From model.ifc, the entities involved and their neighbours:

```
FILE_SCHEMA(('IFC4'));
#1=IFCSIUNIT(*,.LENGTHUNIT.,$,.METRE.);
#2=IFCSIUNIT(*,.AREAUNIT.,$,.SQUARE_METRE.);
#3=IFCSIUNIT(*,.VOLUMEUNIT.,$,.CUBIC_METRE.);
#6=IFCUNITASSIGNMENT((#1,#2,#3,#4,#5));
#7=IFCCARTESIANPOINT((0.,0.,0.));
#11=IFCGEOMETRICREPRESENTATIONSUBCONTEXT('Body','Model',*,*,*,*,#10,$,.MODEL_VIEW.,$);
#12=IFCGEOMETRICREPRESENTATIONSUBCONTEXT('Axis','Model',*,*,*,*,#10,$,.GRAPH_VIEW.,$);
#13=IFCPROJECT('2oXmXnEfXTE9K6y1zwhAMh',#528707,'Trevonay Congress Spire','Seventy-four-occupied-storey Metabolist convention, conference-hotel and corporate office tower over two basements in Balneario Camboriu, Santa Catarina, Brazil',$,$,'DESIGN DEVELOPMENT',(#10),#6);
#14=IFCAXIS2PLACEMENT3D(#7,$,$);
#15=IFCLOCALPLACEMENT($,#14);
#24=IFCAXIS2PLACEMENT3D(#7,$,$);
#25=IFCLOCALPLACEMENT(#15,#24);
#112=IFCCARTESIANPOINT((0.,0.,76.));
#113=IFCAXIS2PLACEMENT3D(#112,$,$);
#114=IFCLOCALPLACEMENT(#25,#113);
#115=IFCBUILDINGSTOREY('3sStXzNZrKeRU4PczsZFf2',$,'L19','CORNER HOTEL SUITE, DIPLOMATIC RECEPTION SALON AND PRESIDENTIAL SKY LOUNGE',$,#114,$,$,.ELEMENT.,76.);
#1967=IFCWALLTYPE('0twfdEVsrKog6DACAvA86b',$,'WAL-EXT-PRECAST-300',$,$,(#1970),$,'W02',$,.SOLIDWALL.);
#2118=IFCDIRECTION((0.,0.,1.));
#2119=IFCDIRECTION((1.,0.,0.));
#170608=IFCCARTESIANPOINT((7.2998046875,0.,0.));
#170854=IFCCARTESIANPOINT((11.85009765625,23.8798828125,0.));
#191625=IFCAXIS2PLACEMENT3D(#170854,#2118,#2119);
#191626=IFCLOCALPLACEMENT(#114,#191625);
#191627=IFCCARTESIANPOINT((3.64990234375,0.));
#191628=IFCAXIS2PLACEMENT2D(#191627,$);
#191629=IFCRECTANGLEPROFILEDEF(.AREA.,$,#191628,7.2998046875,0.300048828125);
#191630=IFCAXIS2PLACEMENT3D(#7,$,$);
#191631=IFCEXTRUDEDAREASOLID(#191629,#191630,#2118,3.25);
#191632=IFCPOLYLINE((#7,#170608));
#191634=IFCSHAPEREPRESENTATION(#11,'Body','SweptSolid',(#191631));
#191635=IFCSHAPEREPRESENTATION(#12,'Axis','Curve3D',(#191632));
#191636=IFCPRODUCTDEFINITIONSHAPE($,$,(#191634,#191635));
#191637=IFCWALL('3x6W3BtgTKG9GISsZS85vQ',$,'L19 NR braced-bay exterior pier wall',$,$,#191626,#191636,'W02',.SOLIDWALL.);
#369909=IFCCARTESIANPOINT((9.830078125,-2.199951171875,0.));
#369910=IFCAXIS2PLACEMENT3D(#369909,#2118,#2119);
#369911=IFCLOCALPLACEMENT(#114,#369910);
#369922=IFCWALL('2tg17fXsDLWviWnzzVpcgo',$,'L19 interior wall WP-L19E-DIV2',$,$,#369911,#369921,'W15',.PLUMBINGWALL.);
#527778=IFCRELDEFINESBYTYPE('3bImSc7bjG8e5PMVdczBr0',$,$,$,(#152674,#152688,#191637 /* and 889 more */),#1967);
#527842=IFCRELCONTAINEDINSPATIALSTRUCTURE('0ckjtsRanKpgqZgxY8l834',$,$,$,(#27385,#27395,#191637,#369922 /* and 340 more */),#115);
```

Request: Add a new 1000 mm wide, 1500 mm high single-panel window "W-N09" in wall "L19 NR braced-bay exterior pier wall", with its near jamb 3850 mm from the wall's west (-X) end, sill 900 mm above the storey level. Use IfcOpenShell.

```python
import numpy as np
import ifcopenshell
import ifcopenshell.api.feature
import ifcopenshell.api.geometry
import ifcopenshell.api.root
import ifcopenshell.api.spatial
import ifcopenshell.geom
import ifcopenshell.util.element
import ifcopenshell.util.placement
import ifcopenshell.util.representation
import ifcopenshell.util.shape
import ifcopenshell.util.unit

model = ifcopenshell.open("model.ifc")
unit_scale = ifcopenshell.util.unit.calculate_unit_scale(model)
settings = ifcopenshell.geom.settings()


def volume(element):
    """Net volume in cubic metres, openings subtracted."""
    shape = ifcopenshell.geom.create_shape(settings, element)
    return ifcopenshell.util.shape.get_volume(shape.geometry)


wall = model.by_guid("3x6W3BtgTKG9GISsZS85vQ")
storey = ifcopenshell.util.element.get_container(wall, ifc_class="IfcBuildingStorey")
context = ifcopenshell.util.representation.get_context(model, "Model", "Body", "MODEL_VIEW")
before = volume(wall)

width, height, from_end, sill = 1, 1.5, 3.85, 0.9  # metres

# The wall runs along its own X axis, and the end named is its -X end.
wall_shape = ifcopenshell.geom.create_shape(settings, wall)
x, y, z = ifcopenshell.util.shape.get_vertices(wall_shape.geometry).T
start = x.min() + from_end
face, thickness = float(y.min()), float(y.max() - y.min())
wall_matrix = ifcopenshell.util.placement.get_local_placement(wall.ObjectPlacement)
level = ifcopenshell.util.placement.get_local_placement(storey.ObjectPlacement)[2, 3]


def in_wall(x, y):
    """Placement at x, y metres in the wall's axes, at sill height."""
    matrix = wall_matrix.copy()
    matrix[:, 3] = wall_matrix @ np.array([x / unit_scale, y / unit_scale, 0.0, 1.0])
    matrix[2, 3] = level + sill / unit_scale
    return matrix


# Opening: a box that overshoots both wall faces by 50 mm.
opening = ifcopenshell.api.root.create_entity(model, ifc_class="IfcOpeningElement", predefined_type="OPENING")
box = ifcopenshell.api.geometry.add_wall_representation(
    model, context=context, length=width, height=height, thickness=thickness + 0.1
)
ifcopenshell.api.geometry.assign_representation(model, product=opening, representation=box)
ifcopenshell.api.geometry.edit_object_placement(model, product=opening, matrix=in_wall(start, face - 0.05), is_si=False)
ifcopenshell.api.feature.add_feature(model, feature=opening, element=wall)

window = ifcopenshell.api.root.create_entity(model, ifc_class="IfcWindow", name="W-N09", predefined_type="WINDOW")
window.OverallWidth, window.OverallHeight = width / unit_scale, height / unit_scale
window.PartitioningType = "SINGLE_PANEL"
body = ifcopenshell.api.geometry.add_window_representation(
    model,
    context=context,
    overall_width=window.OverallWidth,
    overall_height=window.OverallHeight,
    partition_type="SINGLE_PANEL",
)
ifcopenshell.api.geometry.assign_representation(model, product=window, representation=body)
ifcopenshell.api.spatial.assign_container(model, products=[window], relating_structure=storey)
ifcopenshell.api.feature.add_filling(model, opening=opening, element=window)

# Centre the window in the wall's thickness.
ifcopenshell.api.geometry.edit_object_placement(model, product=window, matrix=in_wall(start, face), is_si=False)
window_shape = ifcopenshell.geom.create_shape(settings, window)
depth = ifcopenshell.util.shape.get_vertices(window_shape.geometry)[:, 1]
offset = face + thickness / 2 - (depth.min() + depth.max()) / 2
ifcopenshell.api.geometry.edit_object_placement(model, product=window, matrix=in_wall(start, offset), is_si=False)

after = volume(wall)

print(f"wall volume {before:.3f} -> {after:.3f} m3")

model.write("model_rev.ifc")
```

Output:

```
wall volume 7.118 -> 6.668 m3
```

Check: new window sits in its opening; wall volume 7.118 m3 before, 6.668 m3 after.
